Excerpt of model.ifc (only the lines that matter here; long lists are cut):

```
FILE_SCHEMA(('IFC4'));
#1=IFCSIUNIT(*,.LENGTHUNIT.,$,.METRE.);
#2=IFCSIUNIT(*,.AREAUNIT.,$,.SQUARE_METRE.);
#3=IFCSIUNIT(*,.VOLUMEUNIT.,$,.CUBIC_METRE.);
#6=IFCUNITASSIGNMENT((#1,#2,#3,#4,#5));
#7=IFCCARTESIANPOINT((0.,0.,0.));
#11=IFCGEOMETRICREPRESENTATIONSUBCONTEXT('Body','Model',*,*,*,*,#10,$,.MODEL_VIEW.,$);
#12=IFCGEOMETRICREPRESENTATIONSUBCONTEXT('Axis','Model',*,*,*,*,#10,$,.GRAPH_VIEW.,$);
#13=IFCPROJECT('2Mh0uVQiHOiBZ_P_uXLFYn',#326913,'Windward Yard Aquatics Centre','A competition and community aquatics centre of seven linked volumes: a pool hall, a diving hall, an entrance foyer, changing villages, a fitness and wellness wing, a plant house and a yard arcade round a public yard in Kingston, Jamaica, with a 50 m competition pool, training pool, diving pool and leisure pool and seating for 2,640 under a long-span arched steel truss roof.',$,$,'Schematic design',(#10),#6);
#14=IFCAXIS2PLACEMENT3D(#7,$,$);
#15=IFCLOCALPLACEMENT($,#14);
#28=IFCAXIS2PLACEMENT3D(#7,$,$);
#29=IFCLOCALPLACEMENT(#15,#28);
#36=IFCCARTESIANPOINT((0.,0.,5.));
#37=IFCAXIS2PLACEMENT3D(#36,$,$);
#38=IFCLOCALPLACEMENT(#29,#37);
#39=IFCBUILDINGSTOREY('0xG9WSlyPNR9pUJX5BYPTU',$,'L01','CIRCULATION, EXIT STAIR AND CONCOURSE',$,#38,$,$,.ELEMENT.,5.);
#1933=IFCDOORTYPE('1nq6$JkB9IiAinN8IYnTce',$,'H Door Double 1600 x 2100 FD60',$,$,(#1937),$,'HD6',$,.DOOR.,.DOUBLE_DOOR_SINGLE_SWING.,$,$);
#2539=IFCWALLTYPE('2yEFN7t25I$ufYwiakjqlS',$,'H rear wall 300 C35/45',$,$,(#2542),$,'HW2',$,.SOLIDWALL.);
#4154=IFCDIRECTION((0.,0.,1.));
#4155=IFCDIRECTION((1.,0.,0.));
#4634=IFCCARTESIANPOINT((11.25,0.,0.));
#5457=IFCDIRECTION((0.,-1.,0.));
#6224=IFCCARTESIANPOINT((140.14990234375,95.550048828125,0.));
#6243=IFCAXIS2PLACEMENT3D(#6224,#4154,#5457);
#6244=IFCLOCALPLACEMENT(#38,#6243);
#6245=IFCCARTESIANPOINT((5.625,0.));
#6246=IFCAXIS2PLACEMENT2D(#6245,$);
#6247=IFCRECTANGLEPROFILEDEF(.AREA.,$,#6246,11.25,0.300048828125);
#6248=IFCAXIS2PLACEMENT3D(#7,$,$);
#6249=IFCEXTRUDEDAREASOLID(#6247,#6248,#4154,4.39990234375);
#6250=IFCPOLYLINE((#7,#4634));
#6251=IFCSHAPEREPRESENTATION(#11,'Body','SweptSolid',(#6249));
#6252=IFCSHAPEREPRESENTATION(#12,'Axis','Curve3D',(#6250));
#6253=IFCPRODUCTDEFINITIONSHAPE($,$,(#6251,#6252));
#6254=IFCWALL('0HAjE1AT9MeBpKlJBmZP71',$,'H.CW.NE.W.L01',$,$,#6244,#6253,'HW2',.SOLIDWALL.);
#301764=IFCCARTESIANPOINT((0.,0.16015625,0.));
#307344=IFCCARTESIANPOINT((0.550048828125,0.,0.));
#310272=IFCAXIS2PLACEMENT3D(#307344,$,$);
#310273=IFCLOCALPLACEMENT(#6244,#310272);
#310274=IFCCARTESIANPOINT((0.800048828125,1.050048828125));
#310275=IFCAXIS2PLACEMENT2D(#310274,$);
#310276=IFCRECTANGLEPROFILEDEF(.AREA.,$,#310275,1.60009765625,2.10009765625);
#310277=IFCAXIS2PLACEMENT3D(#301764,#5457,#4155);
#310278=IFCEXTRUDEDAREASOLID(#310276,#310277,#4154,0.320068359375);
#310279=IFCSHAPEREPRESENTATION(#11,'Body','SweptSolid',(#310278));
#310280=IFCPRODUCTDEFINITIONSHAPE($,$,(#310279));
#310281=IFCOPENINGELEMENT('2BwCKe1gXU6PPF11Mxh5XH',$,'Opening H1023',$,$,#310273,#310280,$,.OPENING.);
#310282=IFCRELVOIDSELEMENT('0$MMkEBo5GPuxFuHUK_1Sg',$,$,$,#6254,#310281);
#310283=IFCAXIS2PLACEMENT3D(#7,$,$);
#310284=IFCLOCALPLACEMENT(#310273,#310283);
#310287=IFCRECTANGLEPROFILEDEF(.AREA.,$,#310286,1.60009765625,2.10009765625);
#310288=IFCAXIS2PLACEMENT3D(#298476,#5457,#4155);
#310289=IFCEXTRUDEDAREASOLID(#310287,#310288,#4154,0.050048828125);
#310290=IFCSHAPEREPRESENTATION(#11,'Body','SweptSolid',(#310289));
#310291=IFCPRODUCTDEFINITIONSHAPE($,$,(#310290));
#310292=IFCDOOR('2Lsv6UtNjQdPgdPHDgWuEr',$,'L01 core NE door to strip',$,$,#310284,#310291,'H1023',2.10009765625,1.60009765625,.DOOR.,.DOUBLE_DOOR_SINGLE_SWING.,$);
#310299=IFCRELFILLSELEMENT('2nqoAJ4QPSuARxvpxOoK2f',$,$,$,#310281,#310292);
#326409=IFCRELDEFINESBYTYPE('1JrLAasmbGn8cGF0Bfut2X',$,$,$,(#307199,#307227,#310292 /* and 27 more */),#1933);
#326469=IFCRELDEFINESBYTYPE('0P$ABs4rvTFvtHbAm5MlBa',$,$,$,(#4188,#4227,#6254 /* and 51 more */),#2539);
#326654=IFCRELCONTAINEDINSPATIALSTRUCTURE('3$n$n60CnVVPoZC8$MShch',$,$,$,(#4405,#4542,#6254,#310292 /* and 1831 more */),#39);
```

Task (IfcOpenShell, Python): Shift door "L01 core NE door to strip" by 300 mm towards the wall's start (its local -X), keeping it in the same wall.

```python
import ifcopenshell
import ifcopenshell.api.geometry
import ifcopenshell.util.placement
import ifcopenshell.util.unit

model = ifcopenshell.open("model.ifc")
unit_scale = ifcopenshell.util.unit.calculate_unit_scale(model)

door = model.by_id(310292)
opening = door.FillsVoids[0].RelatingOpeningElement
wall = opening.VoidsElements[0].RelatingBuildingElement

wall_matrix = ifcopenshell.util.placement.get_local_placement(wall.ObjectPlacement)
shift = wall_matrix[:3, 0] * -0.3 / unit_scale
before = ifcopenshell.util.placement.get_local_placement(door.ObjectPlacement)[:3, 3].copy()

# The door is placed relative to its opening, so it follows when the opening moves.
matrix = ifcopenshell.util.placement.get_local_placement(opening.ObjectPlacement)
matrix[:3, 3] += shift
ifcopenshell.api.geometry.edit_object_placement(
    model, product=opening, matrix=matrix, is_si=False, should_transform_children=True
)

after = ifcopenshell.util.placement.get_local_placement(door.ObjectPlacement)[:3, 3]
print("door moved by", (after - before).round(3) + 0.0)

model.write("model-out.ifc")
```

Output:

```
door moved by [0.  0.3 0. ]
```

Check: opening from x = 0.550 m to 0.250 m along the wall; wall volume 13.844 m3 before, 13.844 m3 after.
